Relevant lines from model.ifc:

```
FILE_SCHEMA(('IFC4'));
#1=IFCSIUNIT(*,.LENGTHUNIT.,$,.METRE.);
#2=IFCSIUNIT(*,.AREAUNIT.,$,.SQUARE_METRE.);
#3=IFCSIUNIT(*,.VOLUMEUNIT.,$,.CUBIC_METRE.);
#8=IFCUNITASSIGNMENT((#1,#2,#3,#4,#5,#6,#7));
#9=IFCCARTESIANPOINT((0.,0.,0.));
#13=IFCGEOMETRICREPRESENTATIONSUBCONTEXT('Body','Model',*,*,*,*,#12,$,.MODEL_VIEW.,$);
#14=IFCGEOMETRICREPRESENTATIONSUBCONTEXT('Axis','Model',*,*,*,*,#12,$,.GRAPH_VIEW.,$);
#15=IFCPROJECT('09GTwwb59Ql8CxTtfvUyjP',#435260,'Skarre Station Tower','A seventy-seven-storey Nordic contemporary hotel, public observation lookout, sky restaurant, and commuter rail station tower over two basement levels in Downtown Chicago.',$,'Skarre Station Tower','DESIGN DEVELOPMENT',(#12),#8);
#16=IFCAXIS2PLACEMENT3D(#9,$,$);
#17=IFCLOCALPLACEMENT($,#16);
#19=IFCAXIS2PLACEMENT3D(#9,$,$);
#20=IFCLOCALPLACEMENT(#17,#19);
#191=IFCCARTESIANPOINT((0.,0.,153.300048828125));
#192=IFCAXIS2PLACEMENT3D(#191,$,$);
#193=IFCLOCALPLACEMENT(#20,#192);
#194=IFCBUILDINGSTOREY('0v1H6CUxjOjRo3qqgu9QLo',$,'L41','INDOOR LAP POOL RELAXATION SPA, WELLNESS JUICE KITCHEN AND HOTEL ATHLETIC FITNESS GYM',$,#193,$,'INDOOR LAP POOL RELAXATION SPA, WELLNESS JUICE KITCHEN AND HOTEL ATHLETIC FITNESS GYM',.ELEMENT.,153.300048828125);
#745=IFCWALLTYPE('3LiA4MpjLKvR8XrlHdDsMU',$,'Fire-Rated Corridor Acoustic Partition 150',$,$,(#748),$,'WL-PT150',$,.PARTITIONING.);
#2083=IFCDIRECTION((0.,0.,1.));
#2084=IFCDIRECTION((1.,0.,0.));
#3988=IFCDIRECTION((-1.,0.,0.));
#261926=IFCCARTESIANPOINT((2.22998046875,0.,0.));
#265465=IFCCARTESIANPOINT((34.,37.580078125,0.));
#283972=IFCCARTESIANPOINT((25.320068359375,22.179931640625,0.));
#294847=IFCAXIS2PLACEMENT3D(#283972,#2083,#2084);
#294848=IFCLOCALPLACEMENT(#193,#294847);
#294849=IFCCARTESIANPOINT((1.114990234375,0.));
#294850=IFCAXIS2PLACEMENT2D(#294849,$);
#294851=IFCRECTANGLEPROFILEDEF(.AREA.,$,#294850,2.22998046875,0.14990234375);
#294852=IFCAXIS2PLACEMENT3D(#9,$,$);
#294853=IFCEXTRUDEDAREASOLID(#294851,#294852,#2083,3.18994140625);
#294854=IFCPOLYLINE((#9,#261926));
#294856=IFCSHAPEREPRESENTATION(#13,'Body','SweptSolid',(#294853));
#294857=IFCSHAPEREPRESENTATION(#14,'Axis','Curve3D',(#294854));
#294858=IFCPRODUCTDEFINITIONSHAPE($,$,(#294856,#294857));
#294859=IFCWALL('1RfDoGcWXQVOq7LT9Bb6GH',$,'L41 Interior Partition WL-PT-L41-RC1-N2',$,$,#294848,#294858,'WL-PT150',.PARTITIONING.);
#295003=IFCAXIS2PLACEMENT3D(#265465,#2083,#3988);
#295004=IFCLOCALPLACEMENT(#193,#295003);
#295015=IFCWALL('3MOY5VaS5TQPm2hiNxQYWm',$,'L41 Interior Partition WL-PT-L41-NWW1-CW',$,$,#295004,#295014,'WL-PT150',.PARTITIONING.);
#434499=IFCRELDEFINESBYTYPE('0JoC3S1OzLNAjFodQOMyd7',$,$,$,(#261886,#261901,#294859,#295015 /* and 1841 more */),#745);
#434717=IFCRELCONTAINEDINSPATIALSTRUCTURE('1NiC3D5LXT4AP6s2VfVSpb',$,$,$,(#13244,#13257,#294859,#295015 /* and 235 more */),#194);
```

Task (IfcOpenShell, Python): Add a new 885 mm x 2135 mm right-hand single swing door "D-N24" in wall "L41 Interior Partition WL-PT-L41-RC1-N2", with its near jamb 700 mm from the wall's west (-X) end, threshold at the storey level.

```python
import numpy as np
import ifcopenshell
import ifcopenshell.api.feature
import ifcopenshell.api.geometry
import ifcopenshell.api.root
import ifcopenshell.api.spatial
import ifcopenshell.geom
import ifcopenshell.util.element
import ifcopenshell.util.placement
import ifcopenshell.util.representation
import ifcopenshell.util.shape
import ifcopenshell.util.unit

model = ifcopenshell.open("model.ifc")
unit_scale = ifcopenshell.util.unit.calculate_unit_scale(model)
settings = ifcopenshell.geom.settings()


def volume(element):
    """Net volume in cubic metres, openings subtracted."""
    shape = ifcopenshell.geom.create_shape(settings, element)
    return ifcopenshell.util.shape.get_volume(shape.geometry)


wall = model.by_guid("1RfDoGcWXQVOq7LT9Bb6GH")
storey = ifcopenshell.util.element.get_container(wall, ifc_class="IfcBuildingStorey")
context = ifcopenshell.util.representation.get_context(model, "Model", "Body", "MODEL_VIEW")
before = volume(wall)

width, height, from_end, sill = 0.885, 2.135, 0.7, 0.0  # metres

# The wall runs along its own X axis, and the end named is its -X end.
wall_shape = ifcopenshell.geom.create_shape(settings, wall)
x, y, z = ifcopenshell.util.shape.get_vertices(wall_shape.geometry).T
start = x.min() + from_end
face, thickness = float(y.min()), float(y.max() - y.min())
wall_matrix = ifcopenshell.util.placement.get_local_placement(wall.ObjectPlacement)
level = ifcopenshell.util.placement.get_local_placement(storey.ObjectPlacement)[2, 3]


def in_wall(x, y):
    """Placement at x, y metres in the wall's axes, at sill height."""
    matrix = wall_matrix.copy()
    matrix[:, 3] = wall_matrix @ np.array([x / unit_scale, y / unit_scale, 0.0, 1.0])
    matrix[2, 3] = level + sill / unit_scale
    return matrix


# Opening: a box that overshoots both wall faces by 50 mm.
opening = ifcopenshell.api.root.create_entity(model, ifc_class="IfcOpeningElement", predefined_type="OPENING")
box = ifcopenshell.api.geometry.add_wall_representation(
    model, context=context, length=width, height=height, thickness=thickness + 0.1
)
ifcopenshell.api.geometry.assign_representation(model, product=opening, representation=box)
ifcopenshell.api.geometry.edit_object_placement(model, product=opening, matrix=in_wall(start, face - 0.05), is_si=False)
ifcopenshell.api.feature.add_feature(model, feature=opening, element=wall)

door = ifcopenshell.api.root.create_entity(model, ifc_class="IfcDoor", name="D-N24", predefined_type="DOOR")
door.OverallWidth, door.OverallHeight = width / unit_scale, height / unit_scale
door.OperationType = "SINGLE_SWING_RIGHT"
body = ifcopenshell.api.geometry.add_door_representation(
    model,
    context=context,
    overall_width=door.OverallWidth,
    overall_height=door.OverallHeight,
    operation_type="SINGLE_SWING_RIGHT",
    lining_properties={"LiningDepth": thickness / unit_scale, "ThresholdDepth": thickness / unit_scale},
)
ifcopenshell.api.geometry.assign_representation(model, product=door, representation=body)
ifcopenshell.api.spatial.assign_container(model, products=[door], relating_structure=storey)
ifcopenshell.api.feature.add_filling(model, opening=opening, element=door)

# The lining spans the wall, so the door starts at the wall face.
ifcopenshell.api.geometry.edit_object_placement(model, product=door, matrix=in_wall(start, face), is_si=False)

after = volume(wall)

print(f"wall volume {before:.3f} -> {after:.3f} m3")

model.write("model_updated.ifc")
```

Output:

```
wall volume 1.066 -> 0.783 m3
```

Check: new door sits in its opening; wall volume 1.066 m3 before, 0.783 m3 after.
